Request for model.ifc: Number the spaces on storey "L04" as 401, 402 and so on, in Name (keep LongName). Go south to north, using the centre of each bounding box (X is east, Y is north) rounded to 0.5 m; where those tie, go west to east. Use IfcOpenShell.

First a look at what the model holds.

```python
import ifcopenshell
import ifcopenshell.util.element
import ifcopenshell.util.placement

model = ifcopenshell.open("model.ifc")
print(model.schema)
storey = next(s for s in model.by_type("IfcBuildingStorey") if s.Name == "L04")
spaces = [e for e in ifcopenshell.util.element.get_decomposition(storey) if e.is_a("IfcSpace")]
for e in sorted(spaces, key=lambda e: e.id()):
    origin = ifcopenshell.util.placement.get_local_placement(e.ObjectPlacement)[:3, 3]
    print(e.id(), e.Name, e.LongName, origin.round(2) + 0.0, sep=" | ")
```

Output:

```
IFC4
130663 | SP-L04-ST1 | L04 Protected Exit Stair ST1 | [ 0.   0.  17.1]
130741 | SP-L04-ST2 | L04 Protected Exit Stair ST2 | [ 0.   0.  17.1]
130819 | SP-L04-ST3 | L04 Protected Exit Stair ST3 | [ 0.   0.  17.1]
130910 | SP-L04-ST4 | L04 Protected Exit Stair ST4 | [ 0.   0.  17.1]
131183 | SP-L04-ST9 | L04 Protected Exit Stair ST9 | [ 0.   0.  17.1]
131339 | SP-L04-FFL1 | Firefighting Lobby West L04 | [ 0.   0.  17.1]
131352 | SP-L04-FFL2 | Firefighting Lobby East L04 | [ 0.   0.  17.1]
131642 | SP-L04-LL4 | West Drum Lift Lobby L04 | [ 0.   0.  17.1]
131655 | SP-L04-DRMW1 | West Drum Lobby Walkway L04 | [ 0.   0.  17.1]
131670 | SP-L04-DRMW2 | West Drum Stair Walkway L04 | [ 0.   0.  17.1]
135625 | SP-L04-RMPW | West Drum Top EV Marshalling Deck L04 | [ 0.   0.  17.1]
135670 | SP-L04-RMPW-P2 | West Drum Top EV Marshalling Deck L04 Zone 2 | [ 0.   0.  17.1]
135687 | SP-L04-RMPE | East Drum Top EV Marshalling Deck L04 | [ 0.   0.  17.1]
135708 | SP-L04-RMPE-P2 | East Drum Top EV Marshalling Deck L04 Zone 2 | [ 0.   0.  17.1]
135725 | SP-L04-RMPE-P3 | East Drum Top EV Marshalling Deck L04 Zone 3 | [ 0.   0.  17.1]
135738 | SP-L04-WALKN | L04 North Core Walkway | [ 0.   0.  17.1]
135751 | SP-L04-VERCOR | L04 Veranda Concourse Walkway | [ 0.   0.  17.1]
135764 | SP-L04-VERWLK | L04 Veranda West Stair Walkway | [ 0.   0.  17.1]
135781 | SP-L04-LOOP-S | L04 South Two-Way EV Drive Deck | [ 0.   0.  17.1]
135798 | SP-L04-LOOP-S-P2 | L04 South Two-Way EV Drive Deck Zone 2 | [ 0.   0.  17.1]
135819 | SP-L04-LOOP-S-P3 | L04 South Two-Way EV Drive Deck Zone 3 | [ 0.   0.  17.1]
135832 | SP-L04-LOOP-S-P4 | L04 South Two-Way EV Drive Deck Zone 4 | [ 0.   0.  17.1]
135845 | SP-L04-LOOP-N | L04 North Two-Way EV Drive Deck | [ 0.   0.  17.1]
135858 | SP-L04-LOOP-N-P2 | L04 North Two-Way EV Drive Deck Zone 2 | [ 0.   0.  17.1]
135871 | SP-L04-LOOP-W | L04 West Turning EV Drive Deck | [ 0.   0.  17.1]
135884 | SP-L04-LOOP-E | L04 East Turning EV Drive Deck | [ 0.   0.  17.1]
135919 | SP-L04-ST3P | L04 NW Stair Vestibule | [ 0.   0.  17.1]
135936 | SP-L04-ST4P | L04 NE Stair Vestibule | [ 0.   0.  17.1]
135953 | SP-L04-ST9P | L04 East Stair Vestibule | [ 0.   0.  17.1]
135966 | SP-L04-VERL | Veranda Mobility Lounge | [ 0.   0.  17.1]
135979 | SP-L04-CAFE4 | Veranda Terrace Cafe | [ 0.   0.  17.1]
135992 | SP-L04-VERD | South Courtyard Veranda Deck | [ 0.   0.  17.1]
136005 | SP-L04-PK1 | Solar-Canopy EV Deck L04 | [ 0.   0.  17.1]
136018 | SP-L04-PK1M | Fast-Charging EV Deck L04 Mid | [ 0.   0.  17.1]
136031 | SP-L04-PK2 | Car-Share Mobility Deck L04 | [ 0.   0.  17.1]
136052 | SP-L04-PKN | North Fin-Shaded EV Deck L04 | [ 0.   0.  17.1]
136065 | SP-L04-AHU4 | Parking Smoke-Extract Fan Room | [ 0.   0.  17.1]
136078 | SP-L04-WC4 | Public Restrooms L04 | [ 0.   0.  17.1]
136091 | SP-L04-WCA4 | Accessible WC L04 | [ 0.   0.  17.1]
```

```python
import ifcopenshell
import ifcopenshell.geom
import ifcopenshell.util.element
import ifcopenshell.util.shape

model = ifcopenshell.open("model.ifc")
settings = ifcopenshell.geom.settings()
settings.set("use-world-coords", True)


def centre(element):
    shape = ifcopenshell.geom.create_shape(settings, element)
    return ifcopenshell.util.shape.get_bbox_centroid(shape.geometry)


storey = next(s for s in model.by_type("IfcBuildingStorey") if s.Name == "L04")
spaces = [e for e in ifcopenshell.util.element.get_decomposition(storey) if e.is_a("IfcSpace")]

# Insertion points can sit at a corner or the storey origin, so sort by the geometry (in metres).
centres = {e: centre(e) for e in spaces}
spaces.sort(key=lambda e: (round(centres[e][1] / 0.5), centres[e][0]))

for i, e in enumerate(spaces, start=1):
    number = f"4{i:02d}"
    e.Name = number
    print(e.id(), number)

model.write("model_v2.ifc")
```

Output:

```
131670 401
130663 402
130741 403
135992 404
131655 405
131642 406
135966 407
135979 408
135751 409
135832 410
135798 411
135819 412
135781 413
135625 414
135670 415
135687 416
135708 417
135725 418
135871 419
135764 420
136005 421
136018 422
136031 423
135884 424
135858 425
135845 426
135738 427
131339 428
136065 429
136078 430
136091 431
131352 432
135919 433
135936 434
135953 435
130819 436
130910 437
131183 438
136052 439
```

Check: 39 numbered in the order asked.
